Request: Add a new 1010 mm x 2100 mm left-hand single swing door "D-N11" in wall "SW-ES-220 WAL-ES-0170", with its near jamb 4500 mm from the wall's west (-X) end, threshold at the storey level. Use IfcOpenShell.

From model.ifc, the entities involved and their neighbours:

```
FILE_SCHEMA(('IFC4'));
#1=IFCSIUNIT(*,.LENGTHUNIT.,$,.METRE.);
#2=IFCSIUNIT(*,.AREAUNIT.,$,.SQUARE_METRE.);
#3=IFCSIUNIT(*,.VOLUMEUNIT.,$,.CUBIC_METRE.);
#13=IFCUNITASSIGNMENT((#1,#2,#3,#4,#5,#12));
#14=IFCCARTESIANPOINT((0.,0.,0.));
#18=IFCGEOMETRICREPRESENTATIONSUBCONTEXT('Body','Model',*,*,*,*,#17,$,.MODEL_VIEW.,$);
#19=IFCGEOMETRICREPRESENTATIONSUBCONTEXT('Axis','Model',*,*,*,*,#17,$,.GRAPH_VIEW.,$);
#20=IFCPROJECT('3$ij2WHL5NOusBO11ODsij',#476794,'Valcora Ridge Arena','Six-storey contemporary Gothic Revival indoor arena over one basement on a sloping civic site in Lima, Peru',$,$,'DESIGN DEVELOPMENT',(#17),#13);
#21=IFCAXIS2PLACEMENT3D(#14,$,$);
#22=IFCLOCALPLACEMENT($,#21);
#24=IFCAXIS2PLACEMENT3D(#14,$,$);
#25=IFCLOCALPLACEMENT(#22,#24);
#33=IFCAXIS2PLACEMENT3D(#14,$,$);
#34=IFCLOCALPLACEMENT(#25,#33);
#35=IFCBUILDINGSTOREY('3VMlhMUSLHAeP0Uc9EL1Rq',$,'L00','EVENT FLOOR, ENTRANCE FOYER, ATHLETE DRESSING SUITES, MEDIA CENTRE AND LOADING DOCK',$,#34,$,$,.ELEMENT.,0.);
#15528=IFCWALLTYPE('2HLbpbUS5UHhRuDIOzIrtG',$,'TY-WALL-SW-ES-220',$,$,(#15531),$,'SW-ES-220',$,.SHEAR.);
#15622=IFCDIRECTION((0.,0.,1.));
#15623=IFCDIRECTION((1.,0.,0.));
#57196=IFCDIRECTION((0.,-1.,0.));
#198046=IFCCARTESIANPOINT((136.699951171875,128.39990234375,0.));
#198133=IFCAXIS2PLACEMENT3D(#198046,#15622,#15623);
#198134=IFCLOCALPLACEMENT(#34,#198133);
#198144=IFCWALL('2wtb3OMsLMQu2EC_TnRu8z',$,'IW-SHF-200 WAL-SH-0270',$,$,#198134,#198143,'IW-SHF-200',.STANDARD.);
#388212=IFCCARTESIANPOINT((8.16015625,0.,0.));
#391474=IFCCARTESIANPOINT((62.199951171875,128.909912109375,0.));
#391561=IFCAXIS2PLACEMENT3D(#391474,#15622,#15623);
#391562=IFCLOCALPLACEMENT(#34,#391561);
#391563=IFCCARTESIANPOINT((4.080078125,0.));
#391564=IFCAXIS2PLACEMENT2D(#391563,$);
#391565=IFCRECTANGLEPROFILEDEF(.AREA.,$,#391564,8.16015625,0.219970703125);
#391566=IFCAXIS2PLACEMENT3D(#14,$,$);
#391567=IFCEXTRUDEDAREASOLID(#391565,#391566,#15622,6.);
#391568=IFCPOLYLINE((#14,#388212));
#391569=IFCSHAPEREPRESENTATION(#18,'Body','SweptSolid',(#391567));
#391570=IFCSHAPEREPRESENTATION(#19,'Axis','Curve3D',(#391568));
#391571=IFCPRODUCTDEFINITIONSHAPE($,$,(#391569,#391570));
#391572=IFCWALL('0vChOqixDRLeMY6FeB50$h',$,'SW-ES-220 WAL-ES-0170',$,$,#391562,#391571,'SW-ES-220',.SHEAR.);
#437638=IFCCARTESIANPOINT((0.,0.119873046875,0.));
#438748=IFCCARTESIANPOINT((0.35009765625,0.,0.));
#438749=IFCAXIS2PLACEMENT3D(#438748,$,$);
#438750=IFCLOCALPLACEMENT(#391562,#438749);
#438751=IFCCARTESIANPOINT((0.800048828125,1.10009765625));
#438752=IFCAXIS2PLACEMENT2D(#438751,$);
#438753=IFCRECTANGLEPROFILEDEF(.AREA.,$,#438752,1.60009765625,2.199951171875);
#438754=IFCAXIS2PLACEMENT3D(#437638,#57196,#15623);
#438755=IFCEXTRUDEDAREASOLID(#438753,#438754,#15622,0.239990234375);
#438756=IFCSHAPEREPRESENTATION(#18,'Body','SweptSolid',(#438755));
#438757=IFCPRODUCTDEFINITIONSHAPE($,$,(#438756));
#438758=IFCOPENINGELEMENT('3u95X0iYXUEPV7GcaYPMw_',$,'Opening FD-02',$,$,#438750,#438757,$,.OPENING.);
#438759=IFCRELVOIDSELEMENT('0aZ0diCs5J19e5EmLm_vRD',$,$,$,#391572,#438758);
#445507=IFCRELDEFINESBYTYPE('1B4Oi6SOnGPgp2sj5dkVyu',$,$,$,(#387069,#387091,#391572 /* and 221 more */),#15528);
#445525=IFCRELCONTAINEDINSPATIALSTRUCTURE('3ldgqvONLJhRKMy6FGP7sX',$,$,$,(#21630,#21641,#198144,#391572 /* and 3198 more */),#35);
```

```python
import numpy as np
import ifcopenshell
import ifcopenshell.api.feature
import ifcopenshell.api.geometry
import ifcopenshell.api.root
import ifcopenshell.api.spatial
import ifcopenshell.geom
import ifcopenshell.util.element
import ifcopenshell.util.placement
import ifcopenshell.util.representation
import ifcopenshell.util.shape
import ifcopenshell.util.unit

model = ifcopenshell.open("model.ifc")
unit_scale = ifcopenshell.util.unit.calculate_unit_scale(model)
settings = ifcopenshell.geom.settings()


def volume(element):
    """Net volume in cubic metres, openings subtracted."""
    shape = ifcopenshell.geom.create_shape(settings, element)
    return ifcopenshell.util.shape.get_volume(shape.geometry)


wall = model.by_guid("0vChOqixDRLeMY6FeB50$h")
storey = ifcopenshell.util.element.get_container(wall, ifc_class="IfcBuildingStorey")
context = ifcopenshell.util.representation.get_context(model, "Model", "Body", "MODEL_VIEW")
before = volume(wall)

width, height, from_end, sill = 1.01, 2.1, 4.5, 0.0  # metres

# The wall runs along its own X axis, and the end named is its -X end.
wall_shape = ifcopenshell.geom.create_shape(settings, wall)
x, y, z = ifcopenshell.util.shape.get_vertices(wall_shape.geometry).T
start = x.min() + from_end
face, thickness = float(y.min()), float(y.max() - y.min())
wall_matrix = ifcopenshell.util.placement.get_local_placement(wall.ObjectPlacement)
level = ifcopenshell.util.placement.get_local_placement(storey.ObjectPlacement)[2, 3]


def in_wall(x, y):
    """Placement at x, y metres in the wall's axes, at sill height."""
    matrix = wall_matrix.copy()
    matrix[:, 3] = wall_matrix @ np.array([x / unit_scale, y / unit_scale, 0.0, 1.0])
    matrix[2, 3] = level + sill / unit_scale
    return matrix


# Opening: a box that overshoots both wall faces by 50 mm.
opening = ifcopenshell.api.root.create_entity(model, ifc_class="IfcOpeningElement", predefined_type="OPENING")
box = ifcopenshell.api.geometry.add_wall_representation(
    model, context=context, length=width, height=height, thickness=thickness + 0.1
)
ifcopenshell.api.geometry.assign_representation(model, product=opening, representation=box)
ifcopenshell.api.geometry.edit_object_placement(model, product=opening, matrix=in_wall(start, face - 0.05), is_si=False)
ifcopenshell.api.feature.add_feature(model, feature=opening, element=wall)

door = ifcopenshell.api.root.create_entity(model, ifc_class="IfcDoor", name="D-N11", predefined_type="DOOR")
door.OverallWidth, door.OverallHeight = width / unit_scale, height / unit_scale
door.OperationType = "SINGLE_SWING_LEFT"
body = ifcopenshell.api.geometry.add_door_representation(
    model,
    context=context,
    overall_width=door.OverallWidth,
    overall_height=door.OverallHeight,
    operation_type="SINGLE_SWING_LEFT",
    lining_properties={"LiningDepth": thickness / unit_scale, "ThresholdDepth": thickness / unit_scale},
)
ifcopenshell.api.geometry.assign_representation(model, product=door, representation=body)
ifcopenshell.api.spatial.assign_container(model, products=[door], relating_structure=storey)
ifcopenshell.api.feature.add_filling(model, opening=opening, element=door)

# The lining spans the wall, so the door starts at the wall face.
ifcopenshell.api.geometry.edit_object_placement(model, product=door, matrix=in_wall(start, face), is_si=False)

after = volume(wall)

print(f"wall volume {before:.3f} -> {after:.3f} m3")

model.write("model_rev.ifc")
```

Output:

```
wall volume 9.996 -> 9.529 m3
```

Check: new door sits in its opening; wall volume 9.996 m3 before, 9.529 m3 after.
